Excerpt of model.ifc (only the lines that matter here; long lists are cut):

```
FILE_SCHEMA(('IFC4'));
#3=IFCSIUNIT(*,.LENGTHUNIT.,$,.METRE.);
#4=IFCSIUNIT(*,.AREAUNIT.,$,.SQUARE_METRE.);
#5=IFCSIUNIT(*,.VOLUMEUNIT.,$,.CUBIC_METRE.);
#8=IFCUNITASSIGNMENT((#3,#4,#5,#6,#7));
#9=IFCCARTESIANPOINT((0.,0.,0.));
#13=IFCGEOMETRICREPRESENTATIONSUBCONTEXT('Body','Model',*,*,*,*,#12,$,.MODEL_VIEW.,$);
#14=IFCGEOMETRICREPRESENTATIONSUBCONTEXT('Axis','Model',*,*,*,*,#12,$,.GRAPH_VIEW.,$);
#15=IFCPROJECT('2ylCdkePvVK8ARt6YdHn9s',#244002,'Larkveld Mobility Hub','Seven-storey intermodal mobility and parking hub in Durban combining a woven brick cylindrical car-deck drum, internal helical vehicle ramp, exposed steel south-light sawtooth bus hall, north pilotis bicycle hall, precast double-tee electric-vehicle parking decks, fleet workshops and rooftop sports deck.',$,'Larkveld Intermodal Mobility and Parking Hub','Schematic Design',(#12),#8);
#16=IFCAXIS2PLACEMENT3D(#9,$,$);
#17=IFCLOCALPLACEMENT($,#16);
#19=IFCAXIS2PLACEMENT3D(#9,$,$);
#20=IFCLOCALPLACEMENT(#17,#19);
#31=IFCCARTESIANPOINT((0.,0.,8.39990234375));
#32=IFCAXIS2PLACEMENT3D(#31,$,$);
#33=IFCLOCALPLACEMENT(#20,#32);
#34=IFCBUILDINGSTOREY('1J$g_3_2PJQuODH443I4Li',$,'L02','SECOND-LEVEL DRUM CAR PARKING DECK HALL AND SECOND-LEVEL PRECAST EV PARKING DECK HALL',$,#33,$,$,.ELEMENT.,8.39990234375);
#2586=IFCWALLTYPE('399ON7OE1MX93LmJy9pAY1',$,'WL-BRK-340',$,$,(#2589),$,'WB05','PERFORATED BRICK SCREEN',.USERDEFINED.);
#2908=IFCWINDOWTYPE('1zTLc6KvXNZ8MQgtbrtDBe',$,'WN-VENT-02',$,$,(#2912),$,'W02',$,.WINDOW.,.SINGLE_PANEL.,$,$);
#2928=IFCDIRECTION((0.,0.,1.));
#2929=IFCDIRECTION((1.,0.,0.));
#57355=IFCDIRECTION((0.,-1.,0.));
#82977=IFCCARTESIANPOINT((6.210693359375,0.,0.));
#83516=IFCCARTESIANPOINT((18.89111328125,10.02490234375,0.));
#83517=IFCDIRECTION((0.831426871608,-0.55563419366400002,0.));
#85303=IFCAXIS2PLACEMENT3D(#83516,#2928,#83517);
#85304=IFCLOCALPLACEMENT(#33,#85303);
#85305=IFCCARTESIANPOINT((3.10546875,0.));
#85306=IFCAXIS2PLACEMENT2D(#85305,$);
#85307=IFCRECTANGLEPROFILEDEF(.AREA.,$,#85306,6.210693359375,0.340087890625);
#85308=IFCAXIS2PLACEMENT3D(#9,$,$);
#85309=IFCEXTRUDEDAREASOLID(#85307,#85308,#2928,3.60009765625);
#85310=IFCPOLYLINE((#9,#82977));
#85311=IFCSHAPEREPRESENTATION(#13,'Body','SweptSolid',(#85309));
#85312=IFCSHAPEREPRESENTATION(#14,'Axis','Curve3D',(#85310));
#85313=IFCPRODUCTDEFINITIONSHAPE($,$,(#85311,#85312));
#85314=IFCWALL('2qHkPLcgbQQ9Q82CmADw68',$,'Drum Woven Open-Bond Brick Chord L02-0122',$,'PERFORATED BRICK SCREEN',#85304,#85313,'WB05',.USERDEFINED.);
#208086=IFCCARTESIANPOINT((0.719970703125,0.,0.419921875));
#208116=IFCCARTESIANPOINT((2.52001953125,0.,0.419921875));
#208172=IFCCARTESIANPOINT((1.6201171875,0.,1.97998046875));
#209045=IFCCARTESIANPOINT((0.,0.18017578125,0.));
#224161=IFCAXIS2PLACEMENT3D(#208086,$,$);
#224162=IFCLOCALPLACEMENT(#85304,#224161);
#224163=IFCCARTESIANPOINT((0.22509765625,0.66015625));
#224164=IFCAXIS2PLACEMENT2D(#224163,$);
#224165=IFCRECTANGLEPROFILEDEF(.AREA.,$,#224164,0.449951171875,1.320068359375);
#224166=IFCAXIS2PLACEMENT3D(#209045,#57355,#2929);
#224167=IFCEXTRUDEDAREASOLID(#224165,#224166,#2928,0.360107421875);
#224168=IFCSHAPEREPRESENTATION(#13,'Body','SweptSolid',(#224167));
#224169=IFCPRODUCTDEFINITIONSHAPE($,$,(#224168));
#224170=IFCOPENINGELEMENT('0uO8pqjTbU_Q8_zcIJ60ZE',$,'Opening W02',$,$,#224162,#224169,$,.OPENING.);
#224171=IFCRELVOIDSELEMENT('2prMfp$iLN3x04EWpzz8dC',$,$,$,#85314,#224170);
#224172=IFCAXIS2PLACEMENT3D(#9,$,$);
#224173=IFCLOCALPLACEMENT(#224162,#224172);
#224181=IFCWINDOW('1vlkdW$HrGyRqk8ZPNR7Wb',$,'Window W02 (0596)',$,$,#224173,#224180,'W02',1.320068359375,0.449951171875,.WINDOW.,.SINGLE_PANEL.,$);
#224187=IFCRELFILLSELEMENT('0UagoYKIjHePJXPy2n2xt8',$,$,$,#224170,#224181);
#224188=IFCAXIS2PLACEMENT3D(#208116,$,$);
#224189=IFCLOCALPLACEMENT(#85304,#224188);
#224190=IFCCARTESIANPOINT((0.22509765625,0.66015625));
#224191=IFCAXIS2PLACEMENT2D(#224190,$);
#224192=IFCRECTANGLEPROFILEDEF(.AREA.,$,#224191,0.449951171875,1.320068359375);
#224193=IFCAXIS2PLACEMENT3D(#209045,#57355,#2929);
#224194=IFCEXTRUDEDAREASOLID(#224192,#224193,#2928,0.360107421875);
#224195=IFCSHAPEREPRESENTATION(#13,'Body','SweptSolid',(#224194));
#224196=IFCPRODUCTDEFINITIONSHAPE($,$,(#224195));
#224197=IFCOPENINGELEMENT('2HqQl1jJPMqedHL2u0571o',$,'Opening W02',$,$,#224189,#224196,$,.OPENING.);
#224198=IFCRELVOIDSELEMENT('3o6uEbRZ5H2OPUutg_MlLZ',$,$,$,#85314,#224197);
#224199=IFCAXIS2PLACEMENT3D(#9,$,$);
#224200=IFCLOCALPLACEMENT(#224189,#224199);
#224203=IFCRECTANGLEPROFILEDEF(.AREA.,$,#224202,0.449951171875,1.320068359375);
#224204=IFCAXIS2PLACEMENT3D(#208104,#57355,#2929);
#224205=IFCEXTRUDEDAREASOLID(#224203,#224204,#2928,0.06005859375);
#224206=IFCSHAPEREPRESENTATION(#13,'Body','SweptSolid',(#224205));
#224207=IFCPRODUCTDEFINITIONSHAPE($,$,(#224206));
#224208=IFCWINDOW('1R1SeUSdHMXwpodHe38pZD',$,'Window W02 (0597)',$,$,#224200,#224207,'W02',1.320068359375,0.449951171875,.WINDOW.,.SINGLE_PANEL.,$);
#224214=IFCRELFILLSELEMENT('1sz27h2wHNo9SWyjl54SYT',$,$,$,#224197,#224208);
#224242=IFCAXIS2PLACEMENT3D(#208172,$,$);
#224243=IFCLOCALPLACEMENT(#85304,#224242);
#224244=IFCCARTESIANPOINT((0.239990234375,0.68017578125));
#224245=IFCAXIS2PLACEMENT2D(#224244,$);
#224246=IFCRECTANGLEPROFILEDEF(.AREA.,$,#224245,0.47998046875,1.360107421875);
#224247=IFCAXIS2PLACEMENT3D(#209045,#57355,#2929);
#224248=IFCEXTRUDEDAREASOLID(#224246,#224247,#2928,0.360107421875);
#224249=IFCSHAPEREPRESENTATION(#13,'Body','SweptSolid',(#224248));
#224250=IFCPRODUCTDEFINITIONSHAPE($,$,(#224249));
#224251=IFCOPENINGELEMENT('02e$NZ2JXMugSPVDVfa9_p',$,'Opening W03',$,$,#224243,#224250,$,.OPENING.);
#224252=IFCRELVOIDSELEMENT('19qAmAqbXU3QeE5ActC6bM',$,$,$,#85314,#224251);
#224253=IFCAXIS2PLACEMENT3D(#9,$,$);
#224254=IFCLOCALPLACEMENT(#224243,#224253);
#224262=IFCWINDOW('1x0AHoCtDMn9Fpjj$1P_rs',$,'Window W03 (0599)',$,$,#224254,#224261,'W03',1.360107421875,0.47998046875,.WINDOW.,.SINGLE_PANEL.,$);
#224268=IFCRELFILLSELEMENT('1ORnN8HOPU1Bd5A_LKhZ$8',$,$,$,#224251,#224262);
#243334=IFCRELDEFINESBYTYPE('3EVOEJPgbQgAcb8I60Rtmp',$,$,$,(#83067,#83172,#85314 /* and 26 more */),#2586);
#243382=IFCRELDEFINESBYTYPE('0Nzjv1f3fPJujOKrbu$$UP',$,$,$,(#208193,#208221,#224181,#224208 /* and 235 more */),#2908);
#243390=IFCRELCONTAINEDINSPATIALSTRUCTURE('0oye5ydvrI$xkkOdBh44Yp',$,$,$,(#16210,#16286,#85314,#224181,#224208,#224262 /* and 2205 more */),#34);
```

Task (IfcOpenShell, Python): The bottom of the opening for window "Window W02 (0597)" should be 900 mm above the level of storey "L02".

```python
import numpy as np
import ifcopenshell
import ifcopenshell.api.geometry
import ifcopenshell.geom
import ifcopenshell.util.element
import ifcopenshell.util.placement
import ifcopenshell.util.shape
import ifcopenshell.util.unit

model = ifcopenshell.open("model.ifc")
unit_scale = ifcopenshell.util.unit.calculate_unit_scale(model)

window = model.by_guid("1R1SeUSdHMXwpodHe38pZD")
opening = window.FillsVoids[0].RelatingOpeningElement
storey = ifcopenshell.util.element.get_container(window, ifc_class="IfcBuildingStorey")
level = ifcopenshell.util.placement.get_local_placement(storey.ObjectPlacement)[2, 3]

# The opening's origin need not be at the sill, so measure its lowest point.
shape = ifcopenshell.geom.create_shape(ifcopenshell.geom.settings(), opening)
bottom = ifcopenshell.util.shape.get_shape_bottom_elevation(shape, shape.geometry) / unit_scale
dz = level + 0.9 - bottom

shift = np.array([0.0, 0.0, dz])
# The window is placed relative to its opening, so it follows when the opening moves.
matrix = ifcopenshell.util.placement.get_local_placement(opening.ObjectPlacement)
matrix[:3, 3] += shift
ifcopenshell.api.geometry.edit_object_placement(
    model, product=opening, matrix=matrix, is_si=False, should_transform_children=True
)

print(f"moved by {dz * unit_scale:+.3f} m")

model.write("model-out.ifc")
```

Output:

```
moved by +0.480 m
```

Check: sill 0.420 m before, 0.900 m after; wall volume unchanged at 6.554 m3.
